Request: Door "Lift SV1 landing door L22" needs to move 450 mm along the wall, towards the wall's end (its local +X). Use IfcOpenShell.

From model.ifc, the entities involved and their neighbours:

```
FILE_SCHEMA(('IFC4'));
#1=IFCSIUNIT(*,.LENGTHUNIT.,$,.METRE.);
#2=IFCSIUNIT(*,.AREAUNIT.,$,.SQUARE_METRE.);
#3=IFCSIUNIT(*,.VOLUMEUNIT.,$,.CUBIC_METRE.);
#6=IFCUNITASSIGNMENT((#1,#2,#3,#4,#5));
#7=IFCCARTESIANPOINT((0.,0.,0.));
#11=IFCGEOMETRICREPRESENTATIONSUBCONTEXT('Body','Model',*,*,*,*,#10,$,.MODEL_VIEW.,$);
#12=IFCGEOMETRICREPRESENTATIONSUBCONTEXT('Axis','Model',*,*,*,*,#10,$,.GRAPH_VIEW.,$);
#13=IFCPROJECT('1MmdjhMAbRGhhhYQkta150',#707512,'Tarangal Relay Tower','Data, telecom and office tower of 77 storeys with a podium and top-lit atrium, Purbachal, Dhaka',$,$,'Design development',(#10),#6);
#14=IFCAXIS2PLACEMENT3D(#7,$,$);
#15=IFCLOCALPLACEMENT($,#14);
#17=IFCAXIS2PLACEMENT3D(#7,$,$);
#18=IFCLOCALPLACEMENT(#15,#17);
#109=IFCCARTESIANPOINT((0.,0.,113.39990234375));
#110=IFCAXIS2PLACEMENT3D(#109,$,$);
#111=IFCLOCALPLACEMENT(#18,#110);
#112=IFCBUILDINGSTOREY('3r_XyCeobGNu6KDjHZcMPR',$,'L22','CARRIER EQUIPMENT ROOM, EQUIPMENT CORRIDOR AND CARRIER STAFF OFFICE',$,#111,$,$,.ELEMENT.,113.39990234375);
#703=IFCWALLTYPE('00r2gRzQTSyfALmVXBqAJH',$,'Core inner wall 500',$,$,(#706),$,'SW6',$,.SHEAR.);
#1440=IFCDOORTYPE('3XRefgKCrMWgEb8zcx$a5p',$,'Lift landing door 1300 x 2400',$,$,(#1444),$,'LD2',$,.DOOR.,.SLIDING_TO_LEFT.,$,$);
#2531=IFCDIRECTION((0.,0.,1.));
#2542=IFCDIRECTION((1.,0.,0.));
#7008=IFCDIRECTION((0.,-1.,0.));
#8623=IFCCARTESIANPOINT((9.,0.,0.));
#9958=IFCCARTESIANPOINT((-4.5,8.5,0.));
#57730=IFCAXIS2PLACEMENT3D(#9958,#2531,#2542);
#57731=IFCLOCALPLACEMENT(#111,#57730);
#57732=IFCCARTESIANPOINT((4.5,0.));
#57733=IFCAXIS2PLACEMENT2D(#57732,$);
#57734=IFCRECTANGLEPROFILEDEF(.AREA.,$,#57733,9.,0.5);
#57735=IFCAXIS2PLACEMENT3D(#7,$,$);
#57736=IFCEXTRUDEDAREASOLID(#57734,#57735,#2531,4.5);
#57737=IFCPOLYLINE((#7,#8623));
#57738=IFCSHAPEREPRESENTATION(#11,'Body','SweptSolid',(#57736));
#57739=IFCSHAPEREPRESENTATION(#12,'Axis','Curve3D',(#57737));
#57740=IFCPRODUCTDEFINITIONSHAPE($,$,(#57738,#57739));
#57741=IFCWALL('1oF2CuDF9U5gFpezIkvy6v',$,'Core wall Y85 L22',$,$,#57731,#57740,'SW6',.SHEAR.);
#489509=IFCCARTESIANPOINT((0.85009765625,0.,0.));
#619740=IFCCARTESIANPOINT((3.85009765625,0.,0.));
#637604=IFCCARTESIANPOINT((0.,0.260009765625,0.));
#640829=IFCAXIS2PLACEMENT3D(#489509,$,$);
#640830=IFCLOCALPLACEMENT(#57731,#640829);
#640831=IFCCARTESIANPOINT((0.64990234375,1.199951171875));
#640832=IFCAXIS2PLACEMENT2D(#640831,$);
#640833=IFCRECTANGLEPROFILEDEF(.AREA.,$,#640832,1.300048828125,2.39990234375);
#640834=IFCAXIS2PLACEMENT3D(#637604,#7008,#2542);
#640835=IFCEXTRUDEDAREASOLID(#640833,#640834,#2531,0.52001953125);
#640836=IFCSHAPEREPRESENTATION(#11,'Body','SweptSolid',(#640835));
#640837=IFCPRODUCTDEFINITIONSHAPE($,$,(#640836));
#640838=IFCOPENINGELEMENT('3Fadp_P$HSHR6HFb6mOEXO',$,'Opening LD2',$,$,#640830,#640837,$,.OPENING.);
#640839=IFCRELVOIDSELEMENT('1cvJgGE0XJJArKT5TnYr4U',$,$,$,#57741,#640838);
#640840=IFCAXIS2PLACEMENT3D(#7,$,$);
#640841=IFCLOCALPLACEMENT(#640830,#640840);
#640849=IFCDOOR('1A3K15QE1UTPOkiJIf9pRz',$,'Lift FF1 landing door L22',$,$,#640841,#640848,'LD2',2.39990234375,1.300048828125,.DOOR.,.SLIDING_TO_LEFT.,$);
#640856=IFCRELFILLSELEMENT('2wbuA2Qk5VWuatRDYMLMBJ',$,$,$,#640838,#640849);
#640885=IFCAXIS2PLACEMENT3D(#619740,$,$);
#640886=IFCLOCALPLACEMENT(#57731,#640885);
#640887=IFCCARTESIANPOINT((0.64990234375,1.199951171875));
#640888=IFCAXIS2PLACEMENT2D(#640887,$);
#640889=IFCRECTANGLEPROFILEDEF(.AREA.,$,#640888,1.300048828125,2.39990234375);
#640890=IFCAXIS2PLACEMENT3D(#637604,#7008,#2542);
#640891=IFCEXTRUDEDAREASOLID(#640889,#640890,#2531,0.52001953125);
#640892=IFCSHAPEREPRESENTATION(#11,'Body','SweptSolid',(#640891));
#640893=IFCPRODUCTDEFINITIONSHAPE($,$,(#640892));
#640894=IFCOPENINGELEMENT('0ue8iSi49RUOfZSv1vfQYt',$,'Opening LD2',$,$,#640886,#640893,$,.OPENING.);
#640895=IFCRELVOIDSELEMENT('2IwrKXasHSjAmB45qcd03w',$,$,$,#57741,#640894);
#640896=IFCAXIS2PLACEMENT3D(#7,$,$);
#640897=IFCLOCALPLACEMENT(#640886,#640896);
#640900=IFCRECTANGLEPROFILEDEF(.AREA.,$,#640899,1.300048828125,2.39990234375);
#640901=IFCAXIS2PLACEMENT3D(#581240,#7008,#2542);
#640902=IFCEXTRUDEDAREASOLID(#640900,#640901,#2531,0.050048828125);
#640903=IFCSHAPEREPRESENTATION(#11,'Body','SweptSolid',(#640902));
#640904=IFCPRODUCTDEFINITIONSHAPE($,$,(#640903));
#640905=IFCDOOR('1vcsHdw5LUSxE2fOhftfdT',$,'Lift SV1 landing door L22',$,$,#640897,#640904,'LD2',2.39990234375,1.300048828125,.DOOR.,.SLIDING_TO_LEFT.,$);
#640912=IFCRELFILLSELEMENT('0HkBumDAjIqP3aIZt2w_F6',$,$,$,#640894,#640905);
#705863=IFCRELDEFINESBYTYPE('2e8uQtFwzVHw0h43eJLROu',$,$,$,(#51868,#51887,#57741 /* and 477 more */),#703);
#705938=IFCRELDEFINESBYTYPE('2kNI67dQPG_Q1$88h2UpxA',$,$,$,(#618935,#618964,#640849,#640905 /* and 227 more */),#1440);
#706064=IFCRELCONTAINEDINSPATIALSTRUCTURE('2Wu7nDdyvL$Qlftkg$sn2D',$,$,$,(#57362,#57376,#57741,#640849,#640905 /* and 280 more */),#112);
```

```python
import ifcopenshell
import ifcopenshell.api.geometry
import ifcopenshell.util.placement
import ifcopenshell.util.unit

model = ifcopenshell.open("model.ifc")
unit_scale = ifcopenshell.util.unit.calculate_unit_scale(model)

door = model.by_id(640905)
opening = door.FillsVoids[0].RelatingOpeningElement
wall = opening.VoidsElements[0].RelatingBuildingElement

wall_matrix = ifcopenshell.util.placement.get_local_placement(wall.ObjectPlacement)
shift = wall_matrix[:3, 0] * 0.45 / unit_scale
before = ifcopenshell.util.placement.get_local_placement(door.ObjectPlacement)[:3, 3].copy()

# The door is placed relative to its opening, so it follows when the opening moves.
matrix = ifcopenshell.util.placement.get_local_placement(opening.ObjectPlacement)
matrix[:3, 3] += shift
ifcopenshell.api.geometry.edit_object_placement(
    model, product=opening, matrix=matrix, is_si=False, should_transform_children=True
)

after = ifcopenshell.util.placement.get_local_placement(door.ObjectPlacement)[:3, 3]
print("door moved by", (after - before).round(3) + 0.0)

model.write("model_rev.ifc")
```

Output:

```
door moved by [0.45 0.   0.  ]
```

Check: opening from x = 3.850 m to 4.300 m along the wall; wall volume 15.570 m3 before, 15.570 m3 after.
